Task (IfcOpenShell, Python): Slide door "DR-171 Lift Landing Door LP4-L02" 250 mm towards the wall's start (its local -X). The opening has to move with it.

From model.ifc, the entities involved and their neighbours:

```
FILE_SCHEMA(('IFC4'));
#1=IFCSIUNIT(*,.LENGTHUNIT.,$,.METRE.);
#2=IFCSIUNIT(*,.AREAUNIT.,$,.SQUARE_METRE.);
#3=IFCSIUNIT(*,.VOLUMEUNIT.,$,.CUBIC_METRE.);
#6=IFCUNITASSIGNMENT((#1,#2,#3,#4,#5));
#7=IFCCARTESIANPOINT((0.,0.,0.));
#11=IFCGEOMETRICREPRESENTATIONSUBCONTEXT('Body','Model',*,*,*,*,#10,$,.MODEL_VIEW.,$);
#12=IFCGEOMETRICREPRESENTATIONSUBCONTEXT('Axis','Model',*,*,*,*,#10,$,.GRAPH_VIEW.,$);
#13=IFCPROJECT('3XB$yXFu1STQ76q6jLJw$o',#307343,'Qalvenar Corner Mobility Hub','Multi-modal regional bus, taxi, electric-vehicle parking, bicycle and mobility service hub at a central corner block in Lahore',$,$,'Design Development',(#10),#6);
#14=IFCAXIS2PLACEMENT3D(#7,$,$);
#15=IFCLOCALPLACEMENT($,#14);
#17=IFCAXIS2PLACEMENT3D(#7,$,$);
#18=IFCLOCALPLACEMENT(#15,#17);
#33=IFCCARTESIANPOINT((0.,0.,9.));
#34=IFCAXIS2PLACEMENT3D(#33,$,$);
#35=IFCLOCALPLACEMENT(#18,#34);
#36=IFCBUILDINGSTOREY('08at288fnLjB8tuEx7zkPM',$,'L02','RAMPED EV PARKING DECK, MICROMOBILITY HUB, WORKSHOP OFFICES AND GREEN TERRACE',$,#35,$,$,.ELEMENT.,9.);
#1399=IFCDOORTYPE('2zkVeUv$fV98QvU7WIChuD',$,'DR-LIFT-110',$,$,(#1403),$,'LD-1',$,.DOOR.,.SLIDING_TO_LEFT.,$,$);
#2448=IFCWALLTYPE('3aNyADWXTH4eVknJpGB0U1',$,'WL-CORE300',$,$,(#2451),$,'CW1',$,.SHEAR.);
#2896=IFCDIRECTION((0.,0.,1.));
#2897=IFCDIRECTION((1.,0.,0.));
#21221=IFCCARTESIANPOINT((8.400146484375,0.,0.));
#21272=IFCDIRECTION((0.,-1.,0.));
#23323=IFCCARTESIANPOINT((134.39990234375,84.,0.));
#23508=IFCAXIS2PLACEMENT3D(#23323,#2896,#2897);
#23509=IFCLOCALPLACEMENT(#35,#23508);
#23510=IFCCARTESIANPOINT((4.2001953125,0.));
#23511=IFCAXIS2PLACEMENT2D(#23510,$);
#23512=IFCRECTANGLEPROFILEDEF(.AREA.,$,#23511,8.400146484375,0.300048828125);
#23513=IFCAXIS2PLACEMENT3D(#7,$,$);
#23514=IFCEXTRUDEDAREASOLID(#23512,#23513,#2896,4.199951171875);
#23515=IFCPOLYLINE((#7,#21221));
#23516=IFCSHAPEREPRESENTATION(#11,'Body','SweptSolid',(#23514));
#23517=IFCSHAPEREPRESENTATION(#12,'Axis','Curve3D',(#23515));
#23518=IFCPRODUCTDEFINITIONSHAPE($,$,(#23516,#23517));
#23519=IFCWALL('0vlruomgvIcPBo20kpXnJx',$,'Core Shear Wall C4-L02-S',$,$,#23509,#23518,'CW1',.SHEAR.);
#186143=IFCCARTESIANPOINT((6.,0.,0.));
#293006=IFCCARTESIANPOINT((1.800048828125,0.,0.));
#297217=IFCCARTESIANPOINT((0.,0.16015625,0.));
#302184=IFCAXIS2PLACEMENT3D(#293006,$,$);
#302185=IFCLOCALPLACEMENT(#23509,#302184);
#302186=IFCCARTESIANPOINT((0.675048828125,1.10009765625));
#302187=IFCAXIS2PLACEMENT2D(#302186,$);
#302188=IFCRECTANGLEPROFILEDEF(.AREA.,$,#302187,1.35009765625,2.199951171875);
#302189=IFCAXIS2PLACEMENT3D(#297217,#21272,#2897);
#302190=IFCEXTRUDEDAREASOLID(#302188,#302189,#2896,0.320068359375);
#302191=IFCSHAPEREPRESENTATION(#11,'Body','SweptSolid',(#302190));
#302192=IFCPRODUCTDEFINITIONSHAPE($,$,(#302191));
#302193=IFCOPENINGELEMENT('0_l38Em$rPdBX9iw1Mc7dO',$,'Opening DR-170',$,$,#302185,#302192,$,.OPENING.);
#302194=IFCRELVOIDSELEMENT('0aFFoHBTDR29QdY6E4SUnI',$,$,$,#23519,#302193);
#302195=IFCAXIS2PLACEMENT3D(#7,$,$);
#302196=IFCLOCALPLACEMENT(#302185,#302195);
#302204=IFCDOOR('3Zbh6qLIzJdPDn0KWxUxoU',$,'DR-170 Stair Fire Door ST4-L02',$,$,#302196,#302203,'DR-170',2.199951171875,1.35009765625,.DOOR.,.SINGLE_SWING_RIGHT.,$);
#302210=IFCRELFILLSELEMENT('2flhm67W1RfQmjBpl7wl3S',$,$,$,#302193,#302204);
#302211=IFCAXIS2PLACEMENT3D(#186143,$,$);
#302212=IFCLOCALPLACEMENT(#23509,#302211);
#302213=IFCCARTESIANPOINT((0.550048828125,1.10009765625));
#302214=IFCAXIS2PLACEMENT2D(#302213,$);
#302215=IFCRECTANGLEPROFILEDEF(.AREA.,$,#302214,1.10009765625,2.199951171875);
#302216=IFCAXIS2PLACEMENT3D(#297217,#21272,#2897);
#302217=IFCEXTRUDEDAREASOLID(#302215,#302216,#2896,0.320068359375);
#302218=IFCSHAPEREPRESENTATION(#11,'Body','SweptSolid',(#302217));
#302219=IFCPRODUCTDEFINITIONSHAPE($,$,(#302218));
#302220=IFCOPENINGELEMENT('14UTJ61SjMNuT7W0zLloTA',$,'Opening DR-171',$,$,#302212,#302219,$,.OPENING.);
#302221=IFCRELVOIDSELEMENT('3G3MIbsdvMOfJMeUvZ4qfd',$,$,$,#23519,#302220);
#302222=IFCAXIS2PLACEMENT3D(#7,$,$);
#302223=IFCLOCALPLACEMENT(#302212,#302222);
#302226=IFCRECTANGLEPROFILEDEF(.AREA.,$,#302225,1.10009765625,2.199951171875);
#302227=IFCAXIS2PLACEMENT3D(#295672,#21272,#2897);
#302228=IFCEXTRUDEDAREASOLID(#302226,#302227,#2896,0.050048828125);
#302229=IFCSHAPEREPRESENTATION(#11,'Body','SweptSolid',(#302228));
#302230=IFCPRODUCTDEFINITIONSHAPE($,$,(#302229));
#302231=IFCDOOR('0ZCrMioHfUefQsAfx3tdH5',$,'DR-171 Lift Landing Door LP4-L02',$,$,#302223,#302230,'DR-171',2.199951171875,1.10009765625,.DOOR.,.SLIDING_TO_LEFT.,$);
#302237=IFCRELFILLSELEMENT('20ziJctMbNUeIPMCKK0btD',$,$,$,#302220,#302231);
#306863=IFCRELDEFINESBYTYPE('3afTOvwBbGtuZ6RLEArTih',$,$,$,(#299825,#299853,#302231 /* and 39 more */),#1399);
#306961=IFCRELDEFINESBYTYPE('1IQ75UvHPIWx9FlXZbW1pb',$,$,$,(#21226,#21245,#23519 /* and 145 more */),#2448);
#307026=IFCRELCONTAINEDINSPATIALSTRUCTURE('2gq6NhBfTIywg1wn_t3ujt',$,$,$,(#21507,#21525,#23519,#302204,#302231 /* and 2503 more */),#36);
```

```python
import ifcopenshell
import ifcopenshell.api.geometry
import ifcopenshell.util.placement

model = ifcopenshell.open("model.ifc")

door = model.by_guid("0ZCrMioHfUefQsAfx3tdH5")
opening = door.FillsVoids[0].RelatingOpeningElement
wall = opening.VoidsElements[0].RelatingBuildingElement

wall_matrix = ifcopenshell.util.placement.get_local_placement(wall.ObjectPlacement)
shift = wall_matrix[:3, 0] * -0.25
before = ifcopenshell.util.placement.get_local_placement(door.ObjectPlacement)[:3, 3].copy()

# The door is placed relative to its opening, so it follows when the opening moves.
matrix = ifcopenshell.util.placement.get_local_placement(opening.ObjectPlacement)
matrix[:3, 3] += shift
ifcopenshell.api.geometry.edit_object_placement(
    model, product=opening, matrix=matrix, is_si=False, should_transform_children=True
)

after = ifcopenshell.util.placement.get_local_placement(door.ObjectPlacement)[:3, 3]
print("door moved by", (after - before).round(3) + 0.0)

model.write("model_v2.ifc")
```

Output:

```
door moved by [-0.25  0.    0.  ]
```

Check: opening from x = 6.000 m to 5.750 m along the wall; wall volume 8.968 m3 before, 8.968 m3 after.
